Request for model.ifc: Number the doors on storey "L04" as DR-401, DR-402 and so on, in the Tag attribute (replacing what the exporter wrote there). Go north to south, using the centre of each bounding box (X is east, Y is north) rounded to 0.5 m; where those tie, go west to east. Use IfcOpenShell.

First a look at what the model holds.

```python
import ifcopenshell
import ifcopenshell.util.element
import ifcopenshell.util.placement

model = ifcopenshell.open("model.ifc")
print(model.schema)
storey = next(s for s in model.by_type("IfcBuildingStorey") if s.Name == "L04")
doors = [e for e in ifcopenshell.util.element.get_decomposition(storey) if e.is_a("IfcDoor")]
for e in sorted(doors, key=lambda e: e.id()):
    origin = ifcopenshell.util.placement.get_local_placement(e.ObjectPlacement)[:3, 3]
    print(e.id(), e.Tag, e.Name, origin.round(2) + 0.0, sep=" | ")
```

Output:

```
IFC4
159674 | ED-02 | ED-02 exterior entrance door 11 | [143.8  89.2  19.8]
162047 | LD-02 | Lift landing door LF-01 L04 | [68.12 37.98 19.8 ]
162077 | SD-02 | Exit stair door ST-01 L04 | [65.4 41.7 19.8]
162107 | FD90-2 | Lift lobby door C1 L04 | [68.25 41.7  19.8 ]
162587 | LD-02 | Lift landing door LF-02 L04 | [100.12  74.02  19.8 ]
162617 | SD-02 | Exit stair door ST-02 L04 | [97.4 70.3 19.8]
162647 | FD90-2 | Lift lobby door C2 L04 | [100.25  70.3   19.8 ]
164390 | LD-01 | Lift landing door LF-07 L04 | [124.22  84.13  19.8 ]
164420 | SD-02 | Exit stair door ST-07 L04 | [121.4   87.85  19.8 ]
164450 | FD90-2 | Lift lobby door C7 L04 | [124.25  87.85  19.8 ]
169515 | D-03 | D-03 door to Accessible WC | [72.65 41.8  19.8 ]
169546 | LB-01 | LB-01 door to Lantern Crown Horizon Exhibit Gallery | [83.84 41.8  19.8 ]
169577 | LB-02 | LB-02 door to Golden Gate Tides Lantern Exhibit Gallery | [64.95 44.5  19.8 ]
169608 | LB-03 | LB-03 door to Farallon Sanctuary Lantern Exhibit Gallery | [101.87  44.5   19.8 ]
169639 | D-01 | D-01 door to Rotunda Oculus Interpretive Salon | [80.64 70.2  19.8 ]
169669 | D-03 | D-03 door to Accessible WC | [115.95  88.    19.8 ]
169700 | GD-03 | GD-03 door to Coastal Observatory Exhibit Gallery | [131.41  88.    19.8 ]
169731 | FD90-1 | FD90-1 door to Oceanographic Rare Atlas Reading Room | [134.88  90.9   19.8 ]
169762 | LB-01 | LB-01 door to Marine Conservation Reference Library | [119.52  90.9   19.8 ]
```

```python
import ifcopenshell
import ifcopenshell.geom
import ifcopenshell.util.element
import ifcopenshell.util.shape

model = ifcopenshell.open("model.ifc")
settings = ifcopenshell.geom.settings()
settings.set("use-world-coords", True)


def centre(element):
    shape = ifcopenshell.geom.create_shape(settings, element)
    return ifcopenshell.util.shape.get_bbox_centroid(shape.geometry)


storey = next(s for s in model.by_type("IfcBuildingStorey") if s.Name == "L04")
doors = [e for e in ifcopenshell.util.element.get_decomposition(storey) if e.is_a("IfcDoor")]

# Insertion points can sit at a corner or the storey origin, so sort by the geometry (in metres).
centres = {e: centre(e) for e in doors}
doors.sort(key=lambda e: (-round(centres[e][1] / 0.5), centres[e][0]))

for i, e in enumerate(doors, start=1):
    number = f"DR-4{i:02d}"
    e.Tag = number
    print(e.id(), number)

model.write("model_edited.ifc")
```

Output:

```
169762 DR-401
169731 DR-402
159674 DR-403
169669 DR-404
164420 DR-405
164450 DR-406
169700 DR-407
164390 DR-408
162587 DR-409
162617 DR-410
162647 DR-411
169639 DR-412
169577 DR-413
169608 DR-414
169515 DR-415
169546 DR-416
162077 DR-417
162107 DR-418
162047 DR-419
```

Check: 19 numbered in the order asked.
